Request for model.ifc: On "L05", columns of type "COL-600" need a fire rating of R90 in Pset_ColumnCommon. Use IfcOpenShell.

First a look at what the model holds.

```python
import ifcopenshell
import ifcopenshell.util.element

model = ifcopenshell.open("model.ifc")
print(model.schema)
storey = next(s for s in model.by_type("IfcBuildingStorey") if s.Name == "L05")
columns = [e for e in ifcopenshell.util.element.get_decomposition(storey) if e.is_a("IfcColumn")]
seen = {}
for e in columns:
    element_type = ifcopenshell.util.element.get_type(e)
    key = (element_type.Name if element_type != e and element_type else None, ifcopenshell.util.element.get_pset(e, "Pset_ColumnCommon", "FireRating"))
    seen[key] = seen.get(key, 0) + 1
for (name, value), count in sorted(seen.items(), key=str):
    print(count, "x", name, "|", value)
```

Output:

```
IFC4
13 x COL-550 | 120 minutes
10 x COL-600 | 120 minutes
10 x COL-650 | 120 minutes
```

```python
import ifcopenshell
import ifcopenshell.api.pset
import ifcopenshell.util.element

model = ifcopenshell.open("model.ifc")

storey = next(s for s in model.by_type("IfcBuildingStorey") if s.Name == "L05")
columns = [e for e in ifcopenshell.util.element.get_decomposition(storey) if e.is_a("IfcColumn")]

count = 0
for e in columns:
    element_type = ifcopenshell.util.element.get_type(e)
    if element_type in (None, e) or element_type.Name != "COL-600":
        continue
    # add_pset returns the element's existing set when there is one.
    pset = ifcopenshell.api.pset.add_pset(model, product=e, name="Pset_ColumnCommon")
    ifcopenshell.api.pset.edit_pset(model, pset=pset, properties={"FireRating": "R90"})
    count += 1

print(count, "columns updated")

model.write("model_v2.ifc")
```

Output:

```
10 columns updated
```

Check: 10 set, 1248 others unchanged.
